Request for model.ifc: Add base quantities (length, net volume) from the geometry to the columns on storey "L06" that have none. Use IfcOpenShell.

First a look at what the model holds.

```python
import ifcopenshell
import ifcopenshell.util.element
import ifcopenshell.util.unit

model = ifcopenshell.open("model.ifc")
print(model.schema)
for unit_type in ("LENGTHUNIT", "AREAUNIT", "VOLUMEUNIT"):
    print(unit_type, ifcopenshell.util.unit.calculate_unit_scale(model, unit_type))
storey = next(s for s in model.by_type("IfcBuildingStorey") if s.Name == "L06")
columns = [e for e in ifcopenshell.util.element.get_decomposition(storey) if e.is_a("IfcColumn")]
for e in sorted(columns, key=lambda e: e.id()):
    print(e.id(), e.is_a(), e.Name, list(ifcopenshell.util.element.get_psets(e, qtos_only=True)), sep=" | ")
```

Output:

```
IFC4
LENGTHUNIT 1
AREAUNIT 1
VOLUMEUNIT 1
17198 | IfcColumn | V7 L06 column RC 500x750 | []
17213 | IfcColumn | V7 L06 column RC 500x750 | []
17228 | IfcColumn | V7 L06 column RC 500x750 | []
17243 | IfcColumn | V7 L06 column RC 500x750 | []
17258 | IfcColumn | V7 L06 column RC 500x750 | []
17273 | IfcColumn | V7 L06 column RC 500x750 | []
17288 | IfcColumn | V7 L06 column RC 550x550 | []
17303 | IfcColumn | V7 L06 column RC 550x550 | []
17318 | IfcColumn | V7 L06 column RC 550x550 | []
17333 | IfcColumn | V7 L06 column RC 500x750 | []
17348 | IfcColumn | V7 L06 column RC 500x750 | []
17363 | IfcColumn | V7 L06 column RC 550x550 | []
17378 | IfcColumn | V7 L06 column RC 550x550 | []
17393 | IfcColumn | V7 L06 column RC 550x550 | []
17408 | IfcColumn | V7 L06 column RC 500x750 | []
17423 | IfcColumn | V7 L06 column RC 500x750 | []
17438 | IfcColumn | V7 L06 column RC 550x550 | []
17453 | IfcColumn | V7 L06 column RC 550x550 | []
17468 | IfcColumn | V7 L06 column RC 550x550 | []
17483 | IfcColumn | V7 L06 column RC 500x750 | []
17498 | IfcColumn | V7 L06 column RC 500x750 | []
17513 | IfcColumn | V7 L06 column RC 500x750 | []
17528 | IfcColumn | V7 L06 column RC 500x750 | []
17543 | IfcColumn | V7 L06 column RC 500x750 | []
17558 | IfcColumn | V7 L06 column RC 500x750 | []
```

```python
import ifcopenshell
import ifcopenshell.api.pset
import ifcopenshell.geom
import ifcopenshell.util.element
import ifcopenshell.util.shape
import ifcopenshell.util.unit

model = ifcopenshell.open("model.ifc")
unit_scale = ifcopenshell.util.unit.calculate_unit_scale(model)
volume_scale = ifcopenshell.util.unit.calculate_unit_scale(model, "VOLUMEUNIT")
settings = ifcopenshell.geom.settings()

storey = next(s for s in model.by_type("IfcBuildingStorey") if s.Name == "L06")
columns = [e for e in ifcopenshell.util.element.get_decomposition(storey) if e.is_a("IfcColumn")]

for e in sorted(columns, key=lambda e: e.id()):
    if ifcopenshell.util.element.get_psets(e, qtos_only=True, should_inherit=False):
        continue
    # Geometry comes back in metres, in the element's own axes.
    shape = ifcopenshell.geom.create_shape(settings, e)
    values = {
        "Length": ifcopenshell.util.shape.get_z(shape.geometry) / unit_scale,
        "NetVolume": ifcopenshell.util.shape.get_volume(shape.geometry) / volume_scale,
    }
    qto = ifcopenshell.api.pset.add_qto(model, product=e, name="Qto_ColumnBaseQuantities")
    ifcopenshell.api.pset.edit_qto(model, qto=qto, properties=values)
    print(e.id(), {k: round(v, 3) for k, v in values.items()})

model.write("model_rev.ifc")
```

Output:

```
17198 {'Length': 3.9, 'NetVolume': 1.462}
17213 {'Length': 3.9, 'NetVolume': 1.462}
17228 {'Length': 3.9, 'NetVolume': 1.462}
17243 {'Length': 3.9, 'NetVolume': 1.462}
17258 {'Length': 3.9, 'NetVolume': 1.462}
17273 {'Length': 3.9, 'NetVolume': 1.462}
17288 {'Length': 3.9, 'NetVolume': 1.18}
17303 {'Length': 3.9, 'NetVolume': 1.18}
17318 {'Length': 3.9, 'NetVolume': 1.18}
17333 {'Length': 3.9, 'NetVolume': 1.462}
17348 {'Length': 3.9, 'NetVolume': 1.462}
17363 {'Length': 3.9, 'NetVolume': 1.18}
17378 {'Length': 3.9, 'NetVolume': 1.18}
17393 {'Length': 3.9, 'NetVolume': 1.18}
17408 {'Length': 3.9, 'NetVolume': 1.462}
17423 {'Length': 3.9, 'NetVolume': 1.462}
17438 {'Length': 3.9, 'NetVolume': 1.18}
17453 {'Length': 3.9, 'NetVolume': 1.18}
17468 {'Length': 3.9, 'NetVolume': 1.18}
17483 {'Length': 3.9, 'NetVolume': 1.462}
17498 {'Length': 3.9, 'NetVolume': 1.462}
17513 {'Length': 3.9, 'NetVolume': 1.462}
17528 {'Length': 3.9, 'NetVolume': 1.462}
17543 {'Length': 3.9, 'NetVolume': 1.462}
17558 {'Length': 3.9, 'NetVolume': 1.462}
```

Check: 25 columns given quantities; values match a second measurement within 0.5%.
